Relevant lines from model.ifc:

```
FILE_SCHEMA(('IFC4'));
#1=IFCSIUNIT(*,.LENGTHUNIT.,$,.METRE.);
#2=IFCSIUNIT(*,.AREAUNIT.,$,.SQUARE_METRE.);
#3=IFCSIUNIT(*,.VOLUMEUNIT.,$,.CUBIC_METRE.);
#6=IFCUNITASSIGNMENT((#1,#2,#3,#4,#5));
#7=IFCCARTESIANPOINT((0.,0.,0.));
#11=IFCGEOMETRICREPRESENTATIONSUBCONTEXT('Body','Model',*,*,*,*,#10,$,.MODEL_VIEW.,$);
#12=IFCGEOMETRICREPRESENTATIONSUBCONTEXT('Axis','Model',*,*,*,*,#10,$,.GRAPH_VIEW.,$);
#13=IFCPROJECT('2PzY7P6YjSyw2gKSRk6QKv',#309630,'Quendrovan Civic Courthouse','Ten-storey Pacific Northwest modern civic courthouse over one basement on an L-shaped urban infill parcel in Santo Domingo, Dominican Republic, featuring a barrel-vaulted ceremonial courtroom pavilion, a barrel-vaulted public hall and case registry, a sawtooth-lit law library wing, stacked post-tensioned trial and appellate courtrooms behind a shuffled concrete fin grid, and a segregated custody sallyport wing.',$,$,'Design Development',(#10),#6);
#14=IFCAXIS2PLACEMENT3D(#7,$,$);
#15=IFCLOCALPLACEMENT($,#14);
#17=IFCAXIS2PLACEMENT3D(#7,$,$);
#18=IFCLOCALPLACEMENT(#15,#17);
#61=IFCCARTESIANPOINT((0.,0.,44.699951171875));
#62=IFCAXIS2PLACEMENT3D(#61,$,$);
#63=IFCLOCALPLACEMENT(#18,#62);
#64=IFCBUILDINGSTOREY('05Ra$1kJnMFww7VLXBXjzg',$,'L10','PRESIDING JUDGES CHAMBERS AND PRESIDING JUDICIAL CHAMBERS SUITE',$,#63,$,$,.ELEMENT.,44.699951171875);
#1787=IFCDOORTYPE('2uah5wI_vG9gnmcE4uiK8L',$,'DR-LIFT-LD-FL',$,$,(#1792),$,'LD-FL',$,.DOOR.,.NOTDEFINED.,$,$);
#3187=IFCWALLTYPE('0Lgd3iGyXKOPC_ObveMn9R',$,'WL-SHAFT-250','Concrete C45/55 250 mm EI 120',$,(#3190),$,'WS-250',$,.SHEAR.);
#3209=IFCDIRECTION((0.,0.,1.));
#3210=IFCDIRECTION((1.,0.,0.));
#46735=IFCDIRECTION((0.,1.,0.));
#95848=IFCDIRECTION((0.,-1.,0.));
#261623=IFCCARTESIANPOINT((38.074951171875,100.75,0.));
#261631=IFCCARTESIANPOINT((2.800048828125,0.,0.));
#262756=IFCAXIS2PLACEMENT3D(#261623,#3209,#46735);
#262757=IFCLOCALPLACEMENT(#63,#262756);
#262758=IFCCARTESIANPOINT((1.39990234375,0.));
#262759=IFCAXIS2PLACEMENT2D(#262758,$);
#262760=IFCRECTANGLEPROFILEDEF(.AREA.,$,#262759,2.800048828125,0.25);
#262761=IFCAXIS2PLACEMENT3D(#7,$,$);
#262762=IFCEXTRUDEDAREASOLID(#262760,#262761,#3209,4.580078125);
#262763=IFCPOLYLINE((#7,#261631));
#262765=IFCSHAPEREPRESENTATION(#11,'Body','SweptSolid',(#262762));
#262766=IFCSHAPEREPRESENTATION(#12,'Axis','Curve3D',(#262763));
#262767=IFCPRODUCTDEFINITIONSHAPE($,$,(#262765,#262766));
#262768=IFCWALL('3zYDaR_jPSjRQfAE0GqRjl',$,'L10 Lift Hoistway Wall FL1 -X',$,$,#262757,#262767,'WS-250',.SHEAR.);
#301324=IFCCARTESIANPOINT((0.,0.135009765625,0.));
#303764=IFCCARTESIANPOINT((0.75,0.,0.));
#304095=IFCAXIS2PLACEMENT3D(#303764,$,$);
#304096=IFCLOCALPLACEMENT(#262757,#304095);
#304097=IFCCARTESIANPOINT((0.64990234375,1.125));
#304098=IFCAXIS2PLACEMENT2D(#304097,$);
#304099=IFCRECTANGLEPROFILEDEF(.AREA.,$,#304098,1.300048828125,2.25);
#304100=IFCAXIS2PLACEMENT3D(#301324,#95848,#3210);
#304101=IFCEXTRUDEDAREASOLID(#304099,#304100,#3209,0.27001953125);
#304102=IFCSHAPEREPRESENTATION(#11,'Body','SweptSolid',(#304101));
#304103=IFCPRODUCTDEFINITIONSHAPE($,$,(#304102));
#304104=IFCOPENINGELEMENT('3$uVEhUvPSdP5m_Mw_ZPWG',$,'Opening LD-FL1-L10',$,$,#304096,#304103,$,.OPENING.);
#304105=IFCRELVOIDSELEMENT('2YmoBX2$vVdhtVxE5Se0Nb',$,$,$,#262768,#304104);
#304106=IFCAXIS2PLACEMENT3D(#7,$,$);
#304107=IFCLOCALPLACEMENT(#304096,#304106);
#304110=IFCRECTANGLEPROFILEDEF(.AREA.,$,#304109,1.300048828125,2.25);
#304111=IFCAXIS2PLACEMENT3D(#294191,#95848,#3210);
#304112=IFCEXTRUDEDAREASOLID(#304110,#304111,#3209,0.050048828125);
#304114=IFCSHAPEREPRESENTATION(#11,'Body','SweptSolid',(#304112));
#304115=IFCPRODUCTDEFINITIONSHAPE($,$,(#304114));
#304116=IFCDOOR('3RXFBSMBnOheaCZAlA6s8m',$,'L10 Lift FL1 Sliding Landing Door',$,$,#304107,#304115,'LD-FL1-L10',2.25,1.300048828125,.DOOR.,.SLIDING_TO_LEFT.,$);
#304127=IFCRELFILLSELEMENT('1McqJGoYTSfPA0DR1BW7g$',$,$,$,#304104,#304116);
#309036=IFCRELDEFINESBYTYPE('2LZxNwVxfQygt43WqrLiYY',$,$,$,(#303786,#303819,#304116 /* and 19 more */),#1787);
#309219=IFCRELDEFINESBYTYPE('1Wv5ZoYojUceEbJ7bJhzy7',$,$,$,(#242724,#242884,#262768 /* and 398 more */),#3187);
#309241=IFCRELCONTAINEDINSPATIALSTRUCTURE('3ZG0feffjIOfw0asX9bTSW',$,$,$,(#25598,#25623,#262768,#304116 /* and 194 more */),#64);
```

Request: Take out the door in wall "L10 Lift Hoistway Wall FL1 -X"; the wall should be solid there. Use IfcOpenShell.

```python
import ifcopenshell
import ifcopenshell.api.feature
import ifcopenshell.api.root
import ifcopenshell.geom
import ifcopenshell.util.shape

model = ifcopenshell.open("model.ifc")
settings = ifcopenshell.geom.settings()


def volume(element):
    """Net volume in cubic metres, openings subtracted."""
    shape = ifcopenshell.geom.create_shape(settings, element)
    return ifcopenshell.util.shape.get_volume(shape.geometry)


door = model.by_guid("3RXFBSMBnOheaCZAlA6s8m")
opening = door.FillsVoids[0].RelatingOpeningElement
wall = opening.VoidsElements[0].RelatingBuildingElement
before = volume(wall)

ifcopenshell.api.root.remove_product(model, product=door)
ifcopenshell.api.feature.remove_feature(model, feature=opening)

after = volume(wall)

print(f"wall volume {before:.3f} -> {after:.3f} m3")

model.write("model_edited.ifc")
```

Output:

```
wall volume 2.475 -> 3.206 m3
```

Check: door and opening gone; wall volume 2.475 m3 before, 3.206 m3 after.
